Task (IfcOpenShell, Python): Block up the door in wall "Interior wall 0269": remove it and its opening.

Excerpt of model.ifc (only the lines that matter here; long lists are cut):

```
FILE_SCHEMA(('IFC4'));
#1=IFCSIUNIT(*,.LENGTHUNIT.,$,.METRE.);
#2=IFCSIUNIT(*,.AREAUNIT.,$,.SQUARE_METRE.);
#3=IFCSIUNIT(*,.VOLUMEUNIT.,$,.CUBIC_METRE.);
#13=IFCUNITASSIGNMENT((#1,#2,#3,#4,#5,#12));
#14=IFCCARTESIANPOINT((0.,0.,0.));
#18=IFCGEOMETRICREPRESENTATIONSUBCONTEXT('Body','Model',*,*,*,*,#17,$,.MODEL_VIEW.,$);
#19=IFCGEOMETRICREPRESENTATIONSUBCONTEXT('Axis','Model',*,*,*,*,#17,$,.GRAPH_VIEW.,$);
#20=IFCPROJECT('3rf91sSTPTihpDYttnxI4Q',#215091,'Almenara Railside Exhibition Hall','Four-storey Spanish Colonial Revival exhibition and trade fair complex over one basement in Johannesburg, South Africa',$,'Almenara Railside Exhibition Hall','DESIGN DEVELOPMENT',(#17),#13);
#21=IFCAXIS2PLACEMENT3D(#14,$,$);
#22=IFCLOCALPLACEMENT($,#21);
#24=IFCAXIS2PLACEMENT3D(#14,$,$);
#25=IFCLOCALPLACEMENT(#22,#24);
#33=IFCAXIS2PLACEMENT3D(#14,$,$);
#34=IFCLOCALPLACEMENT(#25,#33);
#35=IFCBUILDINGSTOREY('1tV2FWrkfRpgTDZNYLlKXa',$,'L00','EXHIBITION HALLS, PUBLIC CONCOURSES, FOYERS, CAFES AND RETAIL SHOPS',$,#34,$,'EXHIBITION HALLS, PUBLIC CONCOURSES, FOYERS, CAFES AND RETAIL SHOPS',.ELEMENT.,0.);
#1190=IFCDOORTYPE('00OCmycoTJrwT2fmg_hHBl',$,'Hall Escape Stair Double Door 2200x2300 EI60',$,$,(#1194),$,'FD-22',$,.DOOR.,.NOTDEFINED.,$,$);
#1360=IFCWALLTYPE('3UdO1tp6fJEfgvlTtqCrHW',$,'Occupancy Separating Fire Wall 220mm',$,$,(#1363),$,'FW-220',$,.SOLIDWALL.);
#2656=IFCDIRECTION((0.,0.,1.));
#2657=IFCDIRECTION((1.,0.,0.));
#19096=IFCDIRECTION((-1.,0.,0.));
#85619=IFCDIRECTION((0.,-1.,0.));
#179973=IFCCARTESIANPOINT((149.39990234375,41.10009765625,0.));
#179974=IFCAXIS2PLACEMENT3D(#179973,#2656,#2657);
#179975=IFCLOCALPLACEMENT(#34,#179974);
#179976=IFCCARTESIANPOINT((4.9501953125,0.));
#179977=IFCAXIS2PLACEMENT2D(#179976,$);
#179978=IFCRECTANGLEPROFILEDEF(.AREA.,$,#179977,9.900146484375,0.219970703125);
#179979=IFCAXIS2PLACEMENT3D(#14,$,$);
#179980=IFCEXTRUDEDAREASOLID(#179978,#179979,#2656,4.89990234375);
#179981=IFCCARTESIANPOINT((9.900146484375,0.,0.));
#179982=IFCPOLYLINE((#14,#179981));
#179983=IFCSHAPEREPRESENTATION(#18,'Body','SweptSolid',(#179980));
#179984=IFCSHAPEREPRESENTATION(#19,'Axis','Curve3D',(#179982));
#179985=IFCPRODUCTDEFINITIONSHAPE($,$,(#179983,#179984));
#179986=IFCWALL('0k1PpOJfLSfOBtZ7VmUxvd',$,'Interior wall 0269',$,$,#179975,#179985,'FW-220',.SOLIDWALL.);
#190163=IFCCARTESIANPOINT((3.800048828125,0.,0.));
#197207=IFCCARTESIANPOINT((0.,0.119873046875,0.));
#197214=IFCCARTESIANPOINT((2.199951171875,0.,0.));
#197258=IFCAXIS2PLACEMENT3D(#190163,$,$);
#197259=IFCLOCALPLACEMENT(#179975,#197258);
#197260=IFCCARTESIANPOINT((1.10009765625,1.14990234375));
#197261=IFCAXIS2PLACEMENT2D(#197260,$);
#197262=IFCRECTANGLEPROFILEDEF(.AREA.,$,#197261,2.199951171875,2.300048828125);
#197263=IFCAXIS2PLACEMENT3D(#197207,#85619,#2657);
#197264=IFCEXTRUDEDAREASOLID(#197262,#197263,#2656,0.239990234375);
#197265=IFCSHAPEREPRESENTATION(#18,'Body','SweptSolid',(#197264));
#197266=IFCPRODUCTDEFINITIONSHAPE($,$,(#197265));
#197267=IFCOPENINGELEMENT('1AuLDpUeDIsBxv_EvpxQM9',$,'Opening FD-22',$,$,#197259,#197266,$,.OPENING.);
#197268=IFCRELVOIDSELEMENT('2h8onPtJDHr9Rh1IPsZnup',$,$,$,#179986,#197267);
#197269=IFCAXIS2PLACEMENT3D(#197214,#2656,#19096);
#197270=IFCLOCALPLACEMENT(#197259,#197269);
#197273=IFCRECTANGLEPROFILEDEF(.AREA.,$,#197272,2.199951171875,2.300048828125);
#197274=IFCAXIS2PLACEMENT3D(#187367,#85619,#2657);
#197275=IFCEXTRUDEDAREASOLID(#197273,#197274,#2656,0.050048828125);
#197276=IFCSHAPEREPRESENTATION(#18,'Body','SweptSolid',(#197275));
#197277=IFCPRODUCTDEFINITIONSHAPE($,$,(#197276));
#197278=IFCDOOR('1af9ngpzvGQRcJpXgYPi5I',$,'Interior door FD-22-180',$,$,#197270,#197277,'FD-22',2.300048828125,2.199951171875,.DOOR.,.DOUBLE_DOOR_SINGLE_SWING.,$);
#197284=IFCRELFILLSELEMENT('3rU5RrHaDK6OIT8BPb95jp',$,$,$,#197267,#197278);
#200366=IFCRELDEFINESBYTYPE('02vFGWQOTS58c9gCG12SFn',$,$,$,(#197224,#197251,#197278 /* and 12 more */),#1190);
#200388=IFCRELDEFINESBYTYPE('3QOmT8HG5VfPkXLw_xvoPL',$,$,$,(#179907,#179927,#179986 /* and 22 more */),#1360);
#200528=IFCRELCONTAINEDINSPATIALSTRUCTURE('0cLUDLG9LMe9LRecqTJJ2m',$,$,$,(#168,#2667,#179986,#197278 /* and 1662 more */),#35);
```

```python
import ifcopenshell
import ifcopenshell.api.feature
import ifcopenshell.api.root
import ifcopenshell.geom
import ifcopenshell.util.shape

model = ifcopenshell.open("model.ifc")
settings = ifcopenshell.geom.settings()


def volume(element):
    """Net volume in cubic metres, openings subtracted."""
    shape = ifcopenshell.geom.create_shape(settings, element)
    return ifcopenshell.util.shape.get_volume(shape.geometry)


door = model.by_guid("1af9ngpzvGQRcJpXgYPi5I")
opening = door.FillsVoids[0].RelatingOpeningElement
wall = opening.VoidsElements[0].RelatingBuildingElement
before = volume(wall)

ifcopenshell.api.root.remove_product(model, product=door)
ifcopenshell.api.feature.remove_feature(model, feature=opening)

after = volume(wall)

print(f"wall volume {before:.3f} -> {after:.3f} m3")

model.write("model_rev.ifc")
```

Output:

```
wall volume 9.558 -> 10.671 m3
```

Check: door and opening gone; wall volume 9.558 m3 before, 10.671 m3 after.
